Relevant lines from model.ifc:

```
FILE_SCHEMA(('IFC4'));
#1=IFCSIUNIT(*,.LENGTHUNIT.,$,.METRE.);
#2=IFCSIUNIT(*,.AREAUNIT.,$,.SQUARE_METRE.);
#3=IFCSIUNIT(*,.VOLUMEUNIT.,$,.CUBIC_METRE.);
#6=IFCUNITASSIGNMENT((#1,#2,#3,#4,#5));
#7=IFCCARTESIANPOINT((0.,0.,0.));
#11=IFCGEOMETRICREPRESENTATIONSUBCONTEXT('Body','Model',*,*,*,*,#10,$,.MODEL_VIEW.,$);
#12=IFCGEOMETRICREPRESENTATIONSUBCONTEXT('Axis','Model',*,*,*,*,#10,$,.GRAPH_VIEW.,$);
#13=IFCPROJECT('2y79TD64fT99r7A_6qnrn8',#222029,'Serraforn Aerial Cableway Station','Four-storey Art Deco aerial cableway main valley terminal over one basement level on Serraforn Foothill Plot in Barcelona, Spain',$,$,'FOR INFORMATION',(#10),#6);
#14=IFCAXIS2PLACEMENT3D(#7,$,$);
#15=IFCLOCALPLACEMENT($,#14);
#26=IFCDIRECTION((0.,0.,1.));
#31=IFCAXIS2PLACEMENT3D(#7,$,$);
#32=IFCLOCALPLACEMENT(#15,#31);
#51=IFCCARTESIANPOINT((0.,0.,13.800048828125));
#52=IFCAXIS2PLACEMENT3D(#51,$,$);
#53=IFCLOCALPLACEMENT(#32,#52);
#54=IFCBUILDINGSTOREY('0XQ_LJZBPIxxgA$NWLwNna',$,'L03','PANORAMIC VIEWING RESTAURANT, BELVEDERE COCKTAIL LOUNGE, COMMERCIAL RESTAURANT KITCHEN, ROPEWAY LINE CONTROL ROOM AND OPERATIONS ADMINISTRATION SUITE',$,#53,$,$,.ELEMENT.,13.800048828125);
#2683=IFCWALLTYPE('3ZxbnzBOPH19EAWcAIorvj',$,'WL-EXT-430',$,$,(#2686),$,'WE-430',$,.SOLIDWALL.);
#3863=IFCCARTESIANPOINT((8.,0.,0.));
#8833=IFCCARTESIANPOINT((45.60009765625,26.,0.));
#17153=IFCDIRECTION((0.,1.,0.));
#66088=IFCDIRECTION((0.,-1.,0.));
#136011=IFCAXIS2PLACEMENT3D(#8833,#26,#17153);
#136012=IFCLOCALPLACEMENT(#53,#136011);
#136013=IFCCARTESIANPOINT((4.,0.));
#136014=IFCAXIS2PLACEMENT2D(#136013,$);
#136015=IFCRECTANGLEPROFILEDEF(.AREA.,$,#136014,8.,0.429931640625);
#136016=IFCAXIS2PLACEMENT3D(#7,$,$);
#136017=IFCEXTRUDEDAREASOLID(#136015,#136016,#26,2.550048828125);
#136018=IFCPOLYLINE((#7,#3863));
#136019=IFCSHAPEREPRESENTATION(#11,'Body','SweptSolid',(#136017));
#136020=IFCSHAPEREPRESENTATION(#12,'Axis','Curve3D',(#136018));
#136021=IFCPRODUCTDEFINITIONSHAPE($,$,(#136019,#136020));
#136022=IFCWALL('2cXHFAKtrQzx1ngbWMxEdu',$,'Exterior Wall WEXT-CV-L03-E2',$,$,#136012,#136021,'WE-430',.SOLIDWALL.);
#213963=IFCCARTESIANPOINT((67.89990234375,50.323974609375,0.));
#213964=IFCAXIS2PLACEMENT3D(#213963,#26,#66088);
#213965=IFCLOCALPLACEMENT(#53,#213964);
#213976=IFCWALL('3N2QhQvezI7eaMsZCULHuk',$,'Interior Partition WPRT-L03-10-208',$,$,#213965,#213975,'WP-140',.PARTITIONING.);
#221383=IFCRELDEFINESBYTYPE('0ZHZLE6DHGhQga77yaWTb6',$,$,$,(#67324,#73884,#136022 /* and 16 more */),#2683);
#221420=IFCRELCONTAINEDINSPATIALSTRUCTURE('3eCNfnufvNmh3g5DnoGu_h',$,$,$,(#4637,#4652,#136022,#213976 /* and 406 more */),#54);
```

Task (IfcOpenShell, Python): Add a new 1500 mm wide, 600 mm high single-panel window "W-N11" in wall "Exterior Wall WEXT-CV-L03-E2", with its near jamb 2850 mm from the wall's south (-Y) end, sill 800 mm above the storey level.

```python
import numpy as np
import ifcopenshell
import ifcopenshell.api.feature
import ifcopenshell.api.geometry
import ifcopenshell.api.root
import ifcopenshell.api.spatial
import ifcopenshell.geom
import ifcopenshell.util.element
import ifcopenshell.util.placement
import ifcopenshell.util.representation
import ifcopenshell.util.shape
import ifcopenshell.util.unit

model = ifcopenshell.open("model.ifc")
unit_scale = ifcopenshell.util.unit.calculate_unit_scale(model)
settings = ifcopenshell.geom.settings()


def volume(element):
    """Net volume in cubic metres, openings subtracted."""
    shape = ifcopenshell.geom.create_shape(settings, element)
    return ifcopenshell.util.shape.get_volume(shape.geometry)


wall = model.by_id(136022)
storey = ifcopenshell.util.element.get_container(wall, ifc_class="IfcBuildingStorey")
context = ifcopenshell.util.representation.get_context(model, "Model", "Body", "MODEL_VIEW")
before = volume(wall)

width, height, from_end, sill = 1.5, 0.6, 2.85, 0.8  # metres

# The wall runs along its own X axis, and the end named is its -X end.
wall_shape = ifcopenshell.geom.create_shape(settings, wall)
x, y, z = ifcopenshell.util.shape.get_vertices(wall_shape.geometry).T
start = x.min() + from_end
face, thickness = float(y.min()), float(y.max() - y.min())
wall_matrix = ifcopenshell.util.placement.get_local_placement(wall.ObjectPlacement)
level = ifcopenshell.util.placement.get_local_placement(storey.ObjectPlacement)[2, 3]


def in_wall(x, y):
    """Placement at x, y metres in the wall's axes, at sill height."""
    matrix = wall_matrix.copy()
    matrix[:, 3] = wall_matrix @ np.array([x / unit_scale, y / unit_scale, 0.0, 1.0])
    matrix[2, 3] = level + sill / unit_scale
    return matrix


# Opening: a box that overshoots both wall faces by 50 mm.
opening = ifcopenshell.api.root.create_entity(model, ifc_class="IfcOpeningElement", predefined_type="OPENING")
box = ifcopenshell.api.geometry.add_wall_representation(
    model, context=context, length=width, height=height, thickness=thickness + 0.1
)
ifcopenshell.api.geometry.assign_representation(model, product=opening, representation=box)
ifcopenshell.api.geometry.edit_object_placement(model, product=opening, matrix=in_wall(start, face - 0.05), is_si=False)
ifcopenshell.api.feature.add_feature(model, feature=opening, element=wall)

window = ifcopenshell.api.root.create_entity(model, ifc_class="IfcWindow", name="W-N11", predefined_type="WINDOW")
window.OverallWidth, window.OverallHeight = width / unit_scale, height / unit_scale
window.PartitioningType = "SINGLE_PANEL"
body = ifcopenshell.api.geometry.add_window_representation(
    model,
    context=context,
    overall_width=window.OverallWidth,
    overall_height=window.OverallHeight,
    partition_type="SINGLE_PANEL",
)
ifcopenshell.api.geometry.assign_representation(model, product=window, representation=body)
ifcopenshell.api.spatial.assign_container(model, products=[window], relating_structure=storey)
ifcopenshell.api.feature.add_filling(model, opening=opening, element=window)

# Centre the window in the wall's thickness.
ifcopenshell.api.geometry.edit_object_placement(model, product=window, matrix=in_wall(start, face), is_si=False)
window_shape = ifcopenshell.geom.create_shape(settings, window)
depth = ifcopenshell.util.shape.get_vertices(window_shape.geometry)[:, 1]
offset = face + thickness / 2 - (depth.min() + depth.max()) / 2
ifcopenshell.api.geometry.edit_object_placement(model, product=window, matrix=in_wall(start, offset), is_si=False)

after = volume(wall)

print(f"wall volume {before:.3f} -> {after:.3f} m3")

model.write("model_rev.ifc")
```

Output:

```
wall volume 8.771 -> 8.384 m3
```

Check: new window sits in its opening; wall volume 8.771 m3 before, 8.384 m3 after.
